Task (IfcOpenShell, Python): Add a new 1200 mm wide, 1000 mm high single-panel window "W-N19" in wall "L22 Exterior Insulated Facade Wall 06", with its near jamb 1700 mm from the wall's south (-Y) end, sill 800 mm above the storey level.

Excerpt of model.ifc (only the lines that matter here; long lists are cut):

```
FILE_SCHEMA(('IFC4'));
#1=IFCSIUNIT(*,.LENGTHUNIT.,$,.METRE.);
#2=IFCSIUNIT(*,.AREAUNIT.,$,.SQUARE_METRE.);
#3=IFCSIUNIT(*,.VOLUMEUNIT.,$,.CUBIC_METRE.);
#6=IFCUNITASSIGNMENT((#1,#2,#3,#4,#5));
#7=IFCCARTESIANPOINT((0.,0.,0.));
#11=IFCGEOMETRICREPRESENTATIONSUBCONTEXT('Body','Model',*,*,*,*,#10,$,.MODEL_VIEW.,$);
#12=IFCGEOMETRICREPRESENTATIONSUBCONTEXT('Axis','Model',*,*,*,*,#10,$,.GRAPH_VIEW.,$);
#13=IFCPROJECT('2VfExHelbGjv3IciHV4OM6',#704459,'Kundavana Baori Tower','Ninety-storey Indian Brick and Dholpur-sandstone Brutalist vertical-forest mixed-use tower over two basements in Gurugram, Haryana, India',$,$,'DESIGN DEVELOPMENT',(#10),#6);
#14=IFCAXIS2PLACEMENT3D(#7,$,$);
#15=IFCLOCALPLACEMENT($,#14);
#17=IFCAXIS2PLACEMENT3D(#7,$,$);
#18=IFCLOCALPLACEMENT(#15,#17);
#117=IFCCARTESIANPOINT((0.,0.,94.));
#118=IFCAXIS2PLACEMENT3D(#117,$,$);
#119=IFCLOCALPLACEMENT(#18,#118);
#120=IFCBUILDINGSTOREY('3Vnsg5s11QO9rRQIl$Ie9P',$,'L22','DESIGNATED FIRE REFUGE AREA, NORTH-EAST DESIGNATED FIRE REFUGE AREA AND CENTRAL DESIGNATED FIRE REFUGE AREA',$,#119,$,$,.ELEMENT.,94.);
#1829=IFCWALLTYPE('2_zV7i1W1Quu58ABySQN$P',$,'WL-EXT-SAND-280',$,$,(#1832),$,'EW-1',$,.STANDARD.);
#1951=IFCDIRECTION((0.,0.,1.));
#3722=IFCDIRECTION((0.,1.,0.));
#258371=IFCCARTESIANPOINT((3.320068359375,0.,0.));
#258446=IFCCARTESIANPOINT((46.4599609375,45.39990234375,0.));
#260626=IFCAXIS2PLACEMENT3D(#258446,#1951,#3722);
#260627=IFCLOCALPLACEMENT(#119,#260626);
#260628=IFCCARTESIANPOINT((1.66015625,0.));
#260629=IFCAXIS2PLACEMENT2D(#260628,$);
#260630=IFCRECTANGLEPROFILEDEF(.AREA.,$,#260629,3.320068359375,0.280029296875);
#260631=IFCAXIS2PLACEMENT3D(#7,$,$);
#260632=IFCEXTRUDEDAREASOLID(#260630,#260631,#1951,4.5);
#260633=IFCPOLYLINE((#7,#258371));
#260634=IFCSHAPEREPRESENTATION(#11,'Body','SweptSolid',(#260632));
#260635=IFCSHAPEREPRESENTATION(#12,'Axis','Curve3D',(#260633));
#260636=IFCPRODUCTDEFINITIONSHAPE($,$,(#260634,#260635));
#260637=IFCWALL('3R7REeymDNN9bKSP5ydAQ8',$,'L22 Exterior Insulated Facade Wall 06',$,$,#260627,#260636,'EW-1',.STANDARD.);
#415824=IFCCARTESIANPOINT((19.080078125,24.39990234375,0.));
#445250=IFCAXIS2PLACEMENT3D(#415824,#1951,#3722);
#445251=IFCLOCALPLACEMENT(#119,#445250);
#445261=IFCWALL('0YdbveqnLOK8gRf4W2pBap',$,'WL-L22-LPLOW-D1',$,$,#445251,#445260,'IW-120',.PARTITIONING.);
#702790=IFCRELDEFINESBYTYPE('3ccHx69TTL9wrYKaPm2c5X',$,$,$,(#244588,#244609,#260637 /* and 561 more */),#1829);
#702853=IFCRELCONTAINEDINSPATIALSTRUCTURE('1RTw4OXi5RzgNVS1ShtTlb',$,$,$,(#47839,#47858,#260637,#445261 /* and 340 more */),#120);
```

```python
import numpy as np
import ifcopenshell
import ifcopenshell.api.feature
import ifcopenshell.api.geometry
import ifcopenshell.api.root
import ifcopenshell.api.spatial
import ifcopenshell.geom
import ifcopenshell.util.element
import ifcopenshell.util.placement
import ifcopenshell.util.representation
import ifcopenshell.util.shape
import ifcopenshell.util.unit

model = ifcopenshell.open("model.ifc")
unit_scale = ifcopenshell.util.unit.calculate_unit_scale(model)
settings = ifcopenshell.geom.settings()


def volume(element):
    """Net volume in cubic metres, openings subtracted."""
    shape = ifcopenshell.geom.create_shape(settings, element)
    return ifcopenshell.util.shape.get_volume(shape.geometry)


wall = model.by_guid("3R7REeymDNN9bKSP5ydAQ8")
storey = ifcopenshell.util.element.get_container(wall, ifc_class="IfcBuildingStorey")
context = ifcopenshell.util.representation.get_context(model, "Model", "Body", "MODEL_VIEW")
before = volume(wall)

width, height, from_end, sill = 1.2, 1, 1.7, 0.8  # metres

# The wall runs along its own X axis, and the end named is its -X end.
wall_shape = ifcopenshell.geom.create_shape(settings, wall)
x, y, z = ifcopenshell.util.shape.get_vertices(wall_shape.geometry).T
start = x.min() + from_end
face, thickness = float(y.min()), float(y.max() - y.min())
wall_matrix = ifcopenshell.util.placement.get_local_placement(wall.ObjectPlacement)
level = ifcopenshell.util.placement.get_local_placement(storey.ObjectPlacement)[2, 3]


def in_wall(x, y):
    """Placement at x, y metres in the wall's axes, at sill height."""
    matrix = wall_matrix.copy()
    matrix[:, 3] = wall_matrix @ np.array([x / unit_scale, y / unit_scale, 0.0, 1.0])
    matrix[2, 3] = level + sill / unit_scale
    return matrix


# Opening: a box that overshoots both wall faces by 50 mm.
opening = ifcopenshell.api.root.create_entity(model, ifc_class="IfcOpeningElement", predefined_type="OPENING")
box = ifcopenshell.api.geometry.add_wall_representation(
    model, context=context, length=width, height=height, thickness=thickness + 0.1
)
ifcopenshell.api.geometry.assign_representation(model, product=opening, representation=box)
ifcopenshell.api.geometry.edit_object_placement(model, product=opening, matrix=in_wall(start, face - 0.05), is_si=False)
ifcopenshell.api.feature.add_feature(model, feature=opening, element=wall)

window = ifcopenshell.api.root.create_entity(model, ifc_class="IfcWindow", name="W-N19", predefined_type="WINDOW")
window.OverallWidth, window.OverallHeight = width / unit_scale, height / unit_scale
window.PartitioningType = "SINGLE_PANEL"
body = ifcopenshell.api.geometry.add_window_representation(
    model,
    context=context,
    overall_width=window.OverallWidth,
    overall_height=window.OverallHeight,
    partition_type="SINGLE_PANEL",
)
ifcopenshell.api.geometry.assign_representation(model, product=window, representation=body)
ifcopenshell.api.spatial.assign_container(model, products=[window], relating_structure=storey)
ifcopenshell.api.feature.add_filling(model, opening=opening, element=window)

# Centre the window in the wall's thickness.
ifcopenshell.api.geometry.edit_object_placement(model, product=window, matrix=in_wall(start, face), is_si=False)
window_shape = ifcopenshell.geom.create_shape(settings, window)
depth = ifcopenshell.util.shape.get_vertices(window_shape.geometry)[:, 1]
offset = face + thickness / 2 - (depth.min() + depth.max()) / 2
ifcopenshell.api.geometry.edit_object_placement(model, product=window, matrix=in_wall(start, offset), is_si=False)

after = volume(wall)

print(f"wall volume {before:.3f} -> {after:.3f} m3")

model.write("model_edited.ifc")
```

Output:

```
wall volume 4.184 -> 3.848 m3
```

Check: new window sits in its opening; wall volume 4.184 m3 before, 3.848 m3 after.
